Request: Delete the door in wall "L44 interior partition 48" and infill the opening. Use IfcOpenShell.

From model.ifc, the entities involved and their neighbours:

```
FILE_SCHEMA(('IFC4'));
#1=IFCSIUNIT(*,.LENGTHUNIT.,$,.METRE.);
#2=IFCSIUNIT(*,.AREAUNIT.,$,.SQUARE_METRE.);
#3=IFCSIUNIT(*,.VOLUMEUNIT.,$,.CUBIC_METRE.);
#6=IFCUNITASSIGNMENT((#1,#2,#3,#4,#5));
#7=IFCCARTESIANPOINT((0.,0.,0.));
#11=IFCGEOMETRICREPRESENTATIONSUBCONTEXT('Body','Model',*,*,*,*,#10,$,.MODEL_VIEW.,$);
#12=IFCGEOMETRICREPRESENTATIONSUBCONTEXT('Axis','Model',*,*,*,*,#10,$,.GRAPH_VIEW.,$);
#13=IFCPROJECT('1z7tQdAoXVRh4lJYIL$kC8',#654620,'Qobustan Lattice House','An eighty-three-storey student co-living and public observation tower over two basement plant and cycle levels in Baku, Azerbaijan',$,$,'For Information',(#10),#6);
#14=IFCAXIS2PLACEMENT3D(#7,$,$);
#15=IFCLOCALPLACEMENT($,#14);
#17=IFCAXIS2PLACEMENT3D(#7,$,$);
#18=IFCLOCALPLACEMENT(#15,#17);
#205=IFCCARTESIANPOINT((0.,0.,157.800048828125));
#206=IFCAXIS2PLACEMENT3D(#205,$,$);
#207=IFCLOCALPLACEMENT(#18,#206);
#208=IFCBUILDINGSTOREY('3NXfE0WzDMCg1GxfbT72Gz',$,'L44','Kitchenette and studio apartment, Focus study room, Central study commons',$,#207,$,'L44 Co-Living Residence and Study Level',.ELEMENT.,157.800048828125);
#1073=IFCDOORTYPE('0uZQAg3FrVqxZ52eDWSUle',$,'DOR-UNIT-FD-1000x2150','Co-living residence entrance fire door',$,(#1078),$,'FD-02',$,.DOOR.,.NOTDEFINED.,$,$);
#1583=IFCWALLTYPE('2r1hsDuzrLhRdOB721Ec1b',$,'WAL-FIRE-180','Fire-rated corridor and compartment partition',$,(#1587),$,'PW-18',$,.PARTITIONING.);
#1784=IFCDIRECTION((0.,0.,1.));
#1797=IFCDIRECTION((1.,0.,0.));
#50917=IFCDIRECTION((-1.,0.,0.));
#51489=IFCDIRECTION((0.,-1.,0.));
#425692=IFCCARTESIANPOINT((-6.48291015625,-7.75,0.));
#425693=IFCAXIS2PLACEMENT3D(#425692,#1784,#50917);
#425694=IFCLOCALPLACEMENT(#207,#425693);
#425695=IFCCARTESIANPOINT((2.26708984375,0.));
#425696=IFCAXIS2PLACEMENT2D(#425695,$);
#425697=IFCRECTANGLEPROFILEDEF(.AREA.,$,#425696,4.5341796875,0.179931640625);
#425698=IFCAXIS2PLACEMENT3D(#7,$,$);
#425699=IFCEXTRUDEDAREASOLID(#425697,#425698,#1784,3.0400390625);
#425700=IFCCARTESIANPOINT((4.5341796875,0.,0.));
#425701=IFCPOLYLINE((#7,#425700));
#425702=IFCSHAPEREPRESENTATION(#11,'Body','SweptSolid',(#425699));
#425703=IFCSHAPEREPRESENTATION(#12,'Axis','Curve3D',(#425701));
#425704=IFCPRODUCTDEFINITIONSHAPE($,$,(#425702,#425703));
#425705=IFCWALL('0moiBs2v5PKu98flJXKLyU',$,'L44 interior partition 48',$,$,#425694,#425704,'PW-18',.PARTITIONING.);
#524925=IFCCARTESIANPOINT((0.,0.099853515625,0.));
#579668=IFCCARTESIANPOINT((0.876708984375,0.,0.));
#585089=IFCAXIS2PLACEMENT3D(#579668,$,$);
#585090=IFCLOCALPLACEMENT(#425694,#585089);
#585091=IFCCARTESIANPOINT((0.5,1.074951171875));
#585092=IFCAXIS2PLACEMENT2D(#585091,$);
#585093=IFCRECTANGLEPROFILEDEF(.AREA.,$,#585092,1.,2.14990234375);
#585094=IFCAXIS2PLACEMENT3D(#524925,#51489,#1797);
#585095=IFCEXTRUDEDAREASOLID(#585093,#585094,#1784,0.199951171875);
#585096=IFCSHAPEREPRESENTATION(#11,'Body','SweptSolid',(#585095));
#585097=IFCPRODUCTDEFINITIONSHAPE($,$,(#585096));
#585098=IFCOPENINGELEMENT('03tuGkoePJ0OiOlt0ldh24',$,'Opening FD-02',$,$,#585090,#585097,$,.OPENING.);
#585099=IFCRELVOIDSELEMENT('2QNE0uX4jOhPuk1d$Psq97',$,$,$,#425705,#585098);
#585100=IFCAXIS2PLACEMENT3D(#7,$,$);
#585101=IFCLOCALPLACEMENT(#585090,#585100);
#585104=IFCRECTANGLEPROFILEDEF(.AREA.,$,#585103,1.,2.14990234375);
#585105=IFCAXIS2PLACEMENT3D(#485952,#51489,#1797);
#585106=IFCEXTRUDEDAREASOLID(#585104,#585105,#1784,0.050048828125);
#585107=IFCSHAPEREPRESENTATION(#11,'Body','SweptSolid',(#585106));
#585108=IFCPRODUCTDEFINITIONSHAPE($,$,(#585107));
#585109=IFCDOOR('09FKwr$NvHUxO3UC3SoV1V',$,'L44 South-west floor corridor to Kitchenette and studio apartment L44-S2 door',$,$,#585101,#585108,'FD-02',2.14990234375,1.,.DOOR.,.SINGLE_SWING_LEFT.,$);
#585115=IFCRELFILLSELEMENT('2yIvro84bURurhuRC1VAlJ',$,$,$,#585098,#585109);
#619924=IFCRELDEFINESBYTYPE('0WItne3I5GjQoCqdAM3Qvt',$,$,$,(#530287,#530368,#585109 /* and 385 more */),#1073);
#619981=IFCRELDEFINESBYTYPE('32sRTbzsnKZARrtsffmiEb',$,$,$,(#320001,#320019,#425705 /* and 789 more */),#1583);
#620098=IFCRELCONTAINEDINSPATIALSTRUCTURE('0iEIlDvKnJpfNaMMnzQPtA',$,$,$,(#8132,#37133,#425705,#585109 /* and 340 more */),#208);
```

```python
import ifcopenshell
import ifcopenshell.api.feature
import ifcopenshell.api.root
import ifcopenshell.geom
import ifcopenshell.util.shape

model = ifcopenshell.open("model.ifc")
settings = ifcopenshell.geom.settings()


def volume(element):
    """Net volume in cubic metres, openings subtracted."""
    shape = ifcopenshell.geom.create_shape(settings, element)
    return ifcopenshell.util.shape.get_volume(shape.geometry)


door = model.by_id(585109)
opening = door.FillsVoids[0].RelatingOpeningElement
wall = opening.VoidsElements[0].RelatingBuildingElement
before = volume(wall)

ifcopenshell.api.root.remove_product(model, product=door)
ifcopenshell.api.feature.remove_feature(model, feature=opening)

after = volume(wall)

print(f"wall volume {before:.3f} -> {after:.3f} m3")

model.write("model-out.ifc")
```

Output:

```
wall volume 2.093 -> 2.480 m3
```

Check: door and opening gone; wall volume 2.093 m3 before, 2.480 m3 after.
